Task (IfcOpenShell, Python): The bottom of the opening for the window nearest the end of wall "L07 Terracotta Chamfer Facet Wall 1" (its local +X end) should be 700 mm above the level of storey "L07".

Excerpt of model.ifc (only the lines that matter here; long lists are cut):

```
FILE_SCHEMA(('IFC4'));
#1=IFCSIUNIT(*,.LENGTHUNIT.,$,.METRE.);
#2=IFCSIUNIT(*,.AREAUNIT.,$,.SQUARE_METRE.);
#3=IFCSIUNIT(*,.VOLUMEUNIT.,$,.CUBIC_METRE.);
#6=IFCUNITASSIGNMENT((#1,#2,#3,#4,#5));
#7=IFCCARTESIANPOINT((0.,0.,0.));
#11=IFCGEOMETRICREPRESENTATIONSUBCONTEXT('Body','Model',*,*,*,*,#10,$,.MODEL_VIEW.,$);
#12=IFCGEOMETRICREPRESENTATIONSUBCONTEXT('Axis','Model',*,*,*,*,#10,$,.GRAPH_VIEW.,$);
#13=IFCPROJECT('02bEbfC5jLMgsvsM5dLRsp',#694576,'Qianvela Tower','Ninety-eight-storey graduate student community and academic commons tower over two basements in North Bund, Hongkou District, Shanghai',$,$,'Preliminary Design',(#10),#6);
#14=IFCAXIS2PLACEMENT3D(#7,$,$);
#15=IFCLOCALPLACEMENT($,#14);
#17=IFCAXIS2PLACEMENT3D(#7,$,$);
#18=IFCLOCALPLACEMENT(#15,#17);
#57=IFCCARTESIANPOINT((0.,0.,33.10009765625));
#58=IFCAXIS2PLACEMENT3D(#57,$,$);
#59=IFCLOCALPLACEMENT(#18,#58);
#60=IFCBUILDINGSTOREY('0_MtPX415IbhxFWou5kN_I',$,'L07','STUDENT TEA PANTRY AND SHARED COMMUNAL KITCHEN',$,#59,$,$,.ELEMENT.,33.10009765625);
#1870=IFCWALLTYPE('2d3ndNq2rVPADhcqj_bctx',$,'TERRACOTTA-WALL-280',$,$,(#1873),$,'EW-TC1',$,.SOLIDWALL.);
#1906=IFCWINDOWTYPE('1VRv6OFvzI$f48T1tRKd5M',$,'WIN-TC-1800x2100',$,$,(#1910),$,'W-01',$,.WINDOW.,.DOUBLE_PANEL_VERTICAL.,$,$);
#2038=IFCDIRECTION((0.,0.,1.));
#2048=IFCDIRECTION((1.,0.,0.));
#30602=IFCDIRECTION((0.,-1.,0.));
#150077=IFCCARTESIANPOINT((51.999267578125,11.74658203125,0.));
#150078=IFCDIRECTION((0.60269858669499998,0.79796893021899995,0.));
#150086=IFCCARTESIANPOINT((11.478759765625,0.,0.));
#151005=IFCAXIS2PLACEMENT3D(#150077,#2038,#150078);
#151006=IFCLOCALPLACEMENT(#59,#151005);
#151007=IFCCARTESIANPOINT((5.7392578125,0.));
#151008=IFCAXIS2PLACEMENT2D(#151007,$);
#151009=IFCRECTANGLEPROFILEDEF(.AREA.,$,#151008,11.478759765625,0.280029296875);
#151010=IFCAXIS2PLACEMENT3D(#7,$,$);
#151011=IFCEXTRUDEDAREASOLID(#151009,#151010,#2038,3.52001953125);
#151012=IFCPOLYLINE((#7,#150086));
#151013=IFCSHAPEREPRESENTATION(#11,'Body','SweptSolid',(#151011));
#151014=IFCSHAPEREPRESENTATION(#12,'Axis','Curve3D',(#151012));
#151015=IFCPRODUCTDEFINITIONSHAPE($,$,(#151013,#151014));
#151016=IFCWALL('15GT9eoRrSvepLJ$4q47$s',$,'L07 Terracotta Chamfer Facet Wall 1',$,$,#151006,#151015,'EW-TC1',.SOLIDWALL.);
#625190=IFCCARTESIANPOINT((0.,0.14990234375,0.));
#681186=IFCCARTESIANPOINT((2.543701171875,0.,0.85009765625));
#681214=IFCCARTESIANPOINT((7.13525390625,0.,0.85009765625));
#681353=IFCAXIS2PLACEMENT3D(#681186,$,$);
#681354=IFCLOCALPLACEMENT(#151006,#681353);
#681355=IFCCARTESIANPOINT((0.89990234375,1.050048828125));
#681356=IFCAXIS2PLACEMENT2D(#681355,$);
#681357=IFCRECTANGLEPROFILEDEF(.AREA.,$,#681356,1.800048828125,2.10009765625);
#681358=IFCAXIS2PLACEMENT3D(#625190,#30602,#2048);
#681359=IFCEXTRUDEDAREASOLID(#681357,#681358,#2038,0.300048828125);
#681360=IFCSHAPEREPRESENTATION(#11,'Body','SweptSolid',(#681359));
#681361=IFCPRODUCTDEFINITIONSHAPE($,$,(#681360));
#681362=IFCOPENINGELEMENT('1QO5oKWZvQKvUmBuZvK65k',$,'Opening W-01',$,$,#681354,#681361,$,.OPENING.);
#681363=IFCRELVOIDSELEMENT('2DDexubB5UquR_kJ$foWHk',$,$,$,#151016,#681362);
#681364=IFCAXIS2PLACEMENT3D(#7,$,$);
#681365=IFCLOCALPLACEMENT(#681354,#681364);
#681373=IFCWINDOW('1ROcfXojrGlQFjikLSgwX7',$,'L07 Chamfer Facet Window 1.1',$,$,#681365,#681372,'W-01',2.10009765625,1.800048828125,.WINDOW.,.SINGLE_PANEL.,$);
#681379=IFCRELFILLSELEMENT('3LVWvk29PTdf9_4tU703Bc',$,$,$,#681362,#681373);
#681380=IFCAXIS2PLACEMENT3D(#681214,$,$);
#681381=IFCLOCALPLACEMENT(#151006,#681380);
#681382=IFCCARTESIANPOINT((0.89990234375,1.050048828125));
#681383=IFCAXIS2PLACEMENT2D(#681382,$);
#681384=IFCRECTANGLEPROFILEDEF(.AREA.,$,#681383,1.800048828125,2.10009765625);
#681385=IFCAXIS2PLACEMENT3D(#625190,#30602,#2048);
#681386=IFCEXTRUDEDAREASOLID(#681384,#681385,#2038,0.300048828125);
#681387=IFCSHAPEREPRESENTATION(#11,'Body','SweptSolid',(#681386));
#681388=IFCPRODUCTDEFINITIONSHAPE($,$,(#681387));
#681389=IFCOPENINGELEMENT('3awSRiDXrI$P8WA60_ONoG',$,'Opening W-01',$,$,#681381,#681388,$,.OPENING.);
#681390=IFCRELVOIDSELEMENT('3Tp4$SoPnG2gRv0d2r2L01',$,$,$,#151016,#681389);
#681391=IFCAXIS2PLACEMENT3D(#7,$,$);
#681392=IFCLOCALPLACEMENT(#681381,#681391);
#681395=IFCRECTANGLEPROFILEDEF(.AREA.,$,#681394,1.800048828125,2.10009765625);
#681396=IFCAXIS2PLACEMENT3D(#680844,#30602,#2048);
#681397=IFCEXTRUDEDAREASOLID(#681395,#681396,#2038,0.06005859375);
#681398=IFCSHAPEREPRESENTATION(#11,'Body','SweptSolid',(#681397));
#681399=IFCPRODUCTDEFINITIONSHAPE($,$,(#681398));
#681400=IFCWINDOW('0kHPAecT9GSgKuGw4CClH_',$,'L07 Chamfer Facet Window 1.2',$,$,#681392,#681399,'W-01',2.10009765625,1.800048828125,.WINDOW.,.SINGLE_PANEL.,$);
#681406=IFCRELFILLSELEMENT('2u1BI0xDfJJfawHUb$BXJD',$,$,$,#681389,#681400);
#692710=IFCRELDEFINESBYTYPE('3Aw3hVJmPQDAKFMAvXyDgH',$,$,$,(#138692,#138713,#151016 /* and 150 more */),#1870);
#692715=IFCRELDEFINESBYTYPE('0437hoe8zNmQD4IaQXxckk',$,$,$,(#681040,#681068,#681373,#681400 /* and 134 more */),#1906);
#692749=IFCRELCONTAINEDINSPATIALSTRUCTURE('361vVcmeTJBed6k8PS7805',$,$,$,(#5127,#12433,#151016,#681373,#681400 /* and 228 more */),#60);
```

```python
import numpy as np
import ifcopenshell
import ifcopenshell.api.geometry
import ifcopenshell.geom
import ifcopenshell.util.element
import ifcopenshell.util.placement
import ifcopenshell.util.shape
import ifcopenshell.util.unit

model = ifcopenshell.open("model.ifc")
unit_scale = ifcopenshell.util.unit.calculate_unit_scale(model)

window = model.by_guid("0kHPAecT9GSgKuGw4CClH_")
opening = window.FillsVoids[0].RelatingOpeningElement
storey = ifcopenshell.util.element.get_container(window, ifc_class="IfcBuildingStorey")
level = ifcopenshell.util.placement.get_local_placement(storey.ObjectPlacement)[2, 3]

# The opening's origin need not be at the sill, so measure its lowest point.
shape = ifcopenshell.geom.create_shape(ifcopenshell.geom.settings(), opening)
bottom = ifcopenshell.util.shape.get_shape_bottom_elevation(shape, shape.geometry) / unit_scale
dz = level + 0.7 - bottom

shift = np.array([0.0, 0.0, dz])
# The window is placed relative to its opening, so it follows when the opening moves.
matrix = ifcopenshell.util.placement.get_local_placement(opening.ObjectPlacement)
matrix[:3, 3] += shift
ifcopenshell.api.geometry.edit_object_placement(
    model, product=opening, matrix=matrix, is_si=False, should_transform_children=True
)

print(f"moved by {dz * unit_scale:+.3f} m")

model.write("model_edited.ifc")
```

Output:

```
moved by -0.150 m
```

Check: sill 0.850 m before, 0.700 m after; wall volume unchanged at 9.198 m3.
